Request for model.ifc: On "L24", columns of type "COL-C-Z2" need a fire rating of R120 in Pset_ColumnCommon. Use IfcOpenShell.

First a look at what the model holds.

```python
import ifcopenshell
import ifcopenshell.util.element

model = ifcopenshell.open("model.ifc")
print(model.schema)
storey = next(s for s in model.by_type("IfcBuildingStorey") if s.Name == "L24")
columns = [e for e in ifcopenshell.util.element.get_decomposition(storey) if e.is_a("IfcColumn")]
seen = {}
for e in columns:
    element_type = ifcopenshell.util.element.get_type(e)
    key = (element_type.Name if element_type != e and element_type else None, ifcopenshell.util.element.get_pset(e, "Pset_ColumnCommon", "FireRating"))
    seen[key] = seen.get(key, 0) + 1
for (name, value), count in sorted(seen.items(), key=str):
    print(count, "x", name, "|", value)
```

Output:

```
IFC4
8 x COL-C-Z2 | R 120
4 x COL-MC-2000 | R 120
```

```python
import ifcopenshell
import ifcopenshell.api.pset
import ifcopenshell.util.element

model = ifcopenshell.open("model.ifc")

storey = next(s for s in model.by_type("IfcBuildingStorey") if s.Name == "L24")
columns = [e for e in ifcopenshell.util.element.get_decomposition(storey) if e.is_a("IfcColumn")]

count = 0
for e in columns:
    element_type = ifcopenshell.util.element.get_type(e)
    if element_type in (None, e) or element_type.Name != "COL-C-Z2":
        continue
    # add_pset returns the element's existing set when there is one.
    pset = ifcopenshell.api.pset.add_pset(model, product=e, name="Pset_ColumnCommon")
    ifcopenshell.api.pset.edit_pset(model, pset=pset, properties={"FireRating": "R120"})
    count += 1

print(count, "columns updated")

model.write("model_v2.ifc")
```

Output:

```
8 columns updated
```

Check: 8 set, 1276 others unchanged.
